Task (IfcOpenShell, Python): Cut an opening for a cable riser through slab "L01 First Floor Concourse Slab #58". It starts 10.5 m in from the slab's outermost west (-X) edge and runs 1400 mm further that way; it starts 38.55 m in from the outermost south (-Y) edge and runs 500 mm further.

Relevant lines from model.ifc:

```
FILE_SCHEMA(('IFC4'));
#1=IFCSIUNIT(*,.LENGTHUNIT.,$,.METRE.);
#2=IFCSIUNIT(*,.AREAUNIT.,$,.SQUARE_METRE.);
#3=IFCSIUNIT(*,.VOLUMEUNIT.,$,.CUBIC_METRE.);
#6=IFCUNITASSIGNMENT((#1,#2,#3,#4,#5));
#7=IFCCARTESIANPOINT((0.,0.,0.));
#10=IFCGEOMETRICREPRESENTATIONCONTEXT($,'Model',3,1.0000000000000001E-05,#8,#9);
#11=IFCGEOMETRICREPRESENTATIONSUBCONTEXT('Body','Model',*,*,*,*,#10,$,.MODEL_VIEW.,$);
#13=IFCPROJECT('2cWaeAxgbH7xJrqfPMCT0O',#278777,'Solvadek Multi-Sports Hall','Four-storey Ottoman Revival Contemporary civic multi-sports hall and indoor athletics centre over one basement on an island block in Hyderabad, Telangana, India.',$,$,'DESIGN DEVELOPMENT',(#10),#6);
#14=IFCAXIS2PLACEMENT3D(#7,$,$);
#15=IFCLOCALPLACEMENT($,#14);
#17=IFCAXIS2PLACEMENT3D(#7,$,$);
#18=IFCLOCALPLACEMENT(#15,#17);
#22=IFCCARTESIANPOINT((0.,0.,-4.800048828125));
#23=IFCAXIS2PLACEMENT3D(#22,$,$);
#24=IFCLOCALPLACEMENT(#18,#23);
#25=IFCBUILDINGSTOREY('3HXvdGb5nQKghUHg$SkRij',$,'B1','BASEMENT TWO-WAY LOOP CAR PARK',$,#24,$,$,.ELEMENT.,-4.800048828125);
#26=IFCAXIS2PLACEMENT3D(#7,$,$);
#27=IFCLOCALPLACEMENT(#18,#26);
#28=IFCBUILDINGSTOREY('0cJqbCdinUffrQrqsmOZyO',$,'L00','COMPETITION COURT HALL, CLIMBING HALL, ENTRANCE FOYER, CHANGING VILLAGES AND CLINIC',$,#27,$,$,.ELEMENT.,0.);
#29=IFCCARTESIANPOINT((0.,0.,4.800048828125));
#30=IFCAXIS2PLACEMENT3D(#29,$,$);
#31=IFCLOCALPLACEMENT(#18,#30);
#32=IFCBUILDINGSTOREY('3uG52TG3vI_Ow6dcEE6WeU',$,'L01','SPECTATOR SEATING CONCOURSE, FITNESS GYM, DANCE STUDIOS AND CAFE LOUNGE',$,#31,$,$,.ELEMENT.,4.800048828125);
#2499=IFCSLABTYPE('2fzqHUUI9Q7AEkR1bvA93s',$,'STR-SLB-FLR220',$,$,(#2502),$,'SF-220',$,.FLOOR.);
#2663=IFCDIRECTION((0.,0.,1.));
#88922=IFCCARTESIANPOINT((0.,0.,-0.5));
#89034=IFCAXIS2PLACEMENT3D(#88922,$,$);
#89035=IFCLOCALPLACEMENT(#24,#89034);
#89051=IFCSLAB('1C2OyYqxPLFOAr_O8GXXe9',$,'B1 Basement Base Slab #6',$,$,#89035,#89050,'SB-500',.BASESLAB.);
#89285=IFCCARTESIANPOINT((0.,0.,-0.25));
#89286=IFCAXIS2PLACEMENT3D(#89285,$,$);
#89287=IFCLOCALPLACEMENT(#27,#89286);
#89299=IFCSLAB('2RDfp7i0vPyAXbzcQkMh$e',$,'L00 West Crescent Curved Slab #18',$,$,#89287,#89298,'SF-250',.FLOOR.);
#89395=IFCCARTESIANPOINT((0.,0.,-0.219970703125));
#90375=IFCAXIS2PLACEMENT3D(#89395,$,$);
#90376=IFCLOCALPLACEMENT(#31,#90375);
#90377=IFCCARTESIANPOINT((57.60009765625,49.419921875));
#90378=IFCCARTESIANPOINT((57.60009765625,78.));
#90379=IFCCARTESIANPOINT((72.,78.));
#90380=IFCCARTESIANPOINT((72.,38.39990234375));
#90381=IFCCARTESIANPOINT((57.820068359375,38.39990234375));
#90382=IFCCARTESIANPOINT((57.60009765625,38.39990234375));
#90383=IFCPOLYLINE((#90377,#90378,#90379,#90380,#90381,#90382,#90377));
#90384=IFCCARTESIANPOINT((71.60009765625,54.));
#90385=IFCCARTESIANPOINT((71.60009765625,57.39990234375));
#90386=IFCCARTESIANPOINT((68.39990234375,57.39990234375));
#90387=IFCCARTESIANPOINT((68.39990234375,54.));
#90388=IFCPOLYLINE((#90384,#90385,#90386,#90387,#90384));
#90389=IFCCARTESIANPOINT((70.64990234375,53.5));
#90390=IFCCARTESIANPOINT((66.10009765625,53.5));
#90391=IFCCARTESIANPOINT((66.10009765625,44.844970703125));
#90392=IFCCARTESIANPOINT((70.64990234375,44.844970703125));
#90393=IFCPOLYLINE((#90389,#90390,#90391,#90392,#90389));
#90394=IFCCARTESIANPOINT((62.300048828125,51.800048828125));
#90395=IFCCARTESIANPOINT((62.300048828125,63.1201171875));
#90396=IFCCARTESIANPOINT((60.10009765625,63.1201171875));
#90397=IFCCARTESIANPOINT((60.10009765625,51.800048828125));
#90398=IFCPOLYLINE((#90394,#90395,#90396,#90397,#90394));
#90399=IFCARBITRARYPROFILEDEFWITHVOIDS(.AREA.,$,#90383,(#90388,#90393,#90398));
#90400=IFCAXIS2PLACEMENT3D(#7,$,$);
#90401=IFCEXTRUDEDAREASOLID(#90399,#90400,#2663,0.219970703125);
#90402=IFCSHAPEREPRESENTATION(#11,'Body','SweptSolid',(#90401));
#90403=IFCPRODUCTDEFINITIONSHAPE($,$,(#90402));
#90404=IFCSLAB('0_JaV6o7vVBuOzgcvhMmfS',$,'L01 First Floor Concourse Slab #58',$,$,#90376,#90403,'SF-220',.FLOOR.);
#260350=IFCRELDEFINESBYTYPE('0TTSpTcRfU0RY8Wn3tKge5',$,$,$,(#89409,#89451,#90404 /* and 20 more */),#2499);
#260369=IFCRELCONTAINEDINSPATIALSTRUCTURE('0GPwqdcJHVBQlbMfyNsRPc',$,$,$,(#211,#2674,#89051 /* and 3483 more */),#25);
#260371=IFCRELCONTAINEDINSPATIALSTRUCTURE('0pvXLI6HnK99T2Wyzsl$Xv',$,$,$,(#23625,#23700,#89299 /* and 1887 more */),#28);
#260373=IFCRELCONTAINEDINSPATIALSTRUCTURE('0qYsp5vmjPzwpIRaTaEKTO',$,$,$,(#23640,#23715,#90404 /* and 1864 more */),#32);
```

```python
import numpy as np
import ifcopenshell
import ifcopenshell.api.feature
import ifcopenshell.api.geometry
import ifcopenshell.api.root
import ifcopenshell.geom
import ifcopenshell.util.placement
import ifcopenshell.util.representation
import ifcopenshell.util.shape
import ifcopenshell.util.unit

model = ifcopenshell.open("model.ifc")
unit_scale = ifcopenshell.util.unit.calculate_unit_scale(model)
settings = ifcopenshell.geom.settings()


def volume(element):
    """Net volume in cubic metres, openings subtracted."""
    shape = ifcopenshell.geom.create_shape(settings, element)
    return ifcopenshell.util.shape.get_volume(shape.geometry)


slab = model.by_guid("0_JaV6o7vVBuOzgcvhMmfS")
before = volume(slab)

# Extent in the slab's own axes, in metres. The edges named are its -X and -Y sides.
slab_shape = ifcopenshell.geom.create_shape(settings, slab)
vertices = ifcopenshell.util.shape.get_vertices(slab_shape.geometry)
x_min, y_min, bottom = vertices.min(axis=0)
top = vertices[:, 2].max()

opening = ifcopenshell.api.root.create_entity(model, ifc_class="IfcOpeningElement", name="Cable riser opening", predefined_type="OPENING")
context = ifcopenshell.util.representation.get_context(model, "Model", "Body", "MODEL_VIEW")
width, depth = 1.4, 0.5
outline = [(0.0, 0.0), (width, 0.0), (width, depth), (0.0, depth), (0.0, 0.0)]
# Overshoot both faces by 50 mm so the cut is clean.
shape = ifcopenshell.api.geometry.add_slab_representation(
    model, context=context, depth=top - bottom + 0.1, polyline=outline
)
ifcopenshell.api.geometry.assign_representation(model, product=opening, representation=shape)

matrix = ifcopenshell.util.placement.get_local_placement(slab.ObjectPlacement)
matrix[:, 3] = matrix @ np.append(np.array([x_min + 10.5, y_min + 38.55, bottom - 0.05]) / unit_scale, 1.0)
ifcopenshell.api.geometry.edit_object_placement(model, product=opening, matrix=matrix, is_si=False)
ifcopenshell.api.feature.add_feature(model, feature=opening, element=slab)

after = volume(slab)

print(f"slab volume {before:.3f} -> {after:.3f} m3")

model.write("model_v2.ifc")
```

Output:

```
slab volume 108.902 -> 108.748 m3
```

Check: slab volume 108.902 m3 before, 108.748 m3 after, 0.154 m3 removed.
